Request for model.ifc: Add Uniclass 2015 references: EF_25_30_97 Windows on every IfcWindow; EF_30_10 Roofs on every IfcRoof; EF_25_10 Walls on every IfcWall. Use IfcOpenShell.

First a look at what the model holds.

```python
import ifcopenshell

model = ifcopenshell.open("model.ifc")
print(model.schema)
print("classifications:", [c.Name for c in model.by_type("IfcClassification")])
for ifc_class in ("IfcDoor", "IfcRoof", "IfcStair", "IfcWall", "IfcWindow"):
    print(ifc_class, len(model.by_type(ifc_class)))
```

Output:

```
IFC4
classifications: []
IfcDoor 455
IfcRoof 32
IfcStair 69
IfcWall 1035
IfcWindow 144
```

```python
import ifcopenshell
import ifcopenshell.api.classification

model = ifcopenshell.open("model.ifc")

system = ifcopenshell.api.classification.add_classification(model, classification="Uniclass 2015")

codes = {
    "IfcWindow": ("EF_25_30_97", "Windows"),
    "IfcRoof": ("EF_30_10", "Roofs"),
    "IfcWall": ("EF_25_10", "Walls"),
}
for ifc_class, (code, name) in codes.items():
    products = model.by_type(ifc_class)
    ifcopenshell.api.classification.add_reference(
        model, products=products, classification=system, identification=code, name=name
    )
    print(code, len(products))

model.write("model_updated.ifc")
```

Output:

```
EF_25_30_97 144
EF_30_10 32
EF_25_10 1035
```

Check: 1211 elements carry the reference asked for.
